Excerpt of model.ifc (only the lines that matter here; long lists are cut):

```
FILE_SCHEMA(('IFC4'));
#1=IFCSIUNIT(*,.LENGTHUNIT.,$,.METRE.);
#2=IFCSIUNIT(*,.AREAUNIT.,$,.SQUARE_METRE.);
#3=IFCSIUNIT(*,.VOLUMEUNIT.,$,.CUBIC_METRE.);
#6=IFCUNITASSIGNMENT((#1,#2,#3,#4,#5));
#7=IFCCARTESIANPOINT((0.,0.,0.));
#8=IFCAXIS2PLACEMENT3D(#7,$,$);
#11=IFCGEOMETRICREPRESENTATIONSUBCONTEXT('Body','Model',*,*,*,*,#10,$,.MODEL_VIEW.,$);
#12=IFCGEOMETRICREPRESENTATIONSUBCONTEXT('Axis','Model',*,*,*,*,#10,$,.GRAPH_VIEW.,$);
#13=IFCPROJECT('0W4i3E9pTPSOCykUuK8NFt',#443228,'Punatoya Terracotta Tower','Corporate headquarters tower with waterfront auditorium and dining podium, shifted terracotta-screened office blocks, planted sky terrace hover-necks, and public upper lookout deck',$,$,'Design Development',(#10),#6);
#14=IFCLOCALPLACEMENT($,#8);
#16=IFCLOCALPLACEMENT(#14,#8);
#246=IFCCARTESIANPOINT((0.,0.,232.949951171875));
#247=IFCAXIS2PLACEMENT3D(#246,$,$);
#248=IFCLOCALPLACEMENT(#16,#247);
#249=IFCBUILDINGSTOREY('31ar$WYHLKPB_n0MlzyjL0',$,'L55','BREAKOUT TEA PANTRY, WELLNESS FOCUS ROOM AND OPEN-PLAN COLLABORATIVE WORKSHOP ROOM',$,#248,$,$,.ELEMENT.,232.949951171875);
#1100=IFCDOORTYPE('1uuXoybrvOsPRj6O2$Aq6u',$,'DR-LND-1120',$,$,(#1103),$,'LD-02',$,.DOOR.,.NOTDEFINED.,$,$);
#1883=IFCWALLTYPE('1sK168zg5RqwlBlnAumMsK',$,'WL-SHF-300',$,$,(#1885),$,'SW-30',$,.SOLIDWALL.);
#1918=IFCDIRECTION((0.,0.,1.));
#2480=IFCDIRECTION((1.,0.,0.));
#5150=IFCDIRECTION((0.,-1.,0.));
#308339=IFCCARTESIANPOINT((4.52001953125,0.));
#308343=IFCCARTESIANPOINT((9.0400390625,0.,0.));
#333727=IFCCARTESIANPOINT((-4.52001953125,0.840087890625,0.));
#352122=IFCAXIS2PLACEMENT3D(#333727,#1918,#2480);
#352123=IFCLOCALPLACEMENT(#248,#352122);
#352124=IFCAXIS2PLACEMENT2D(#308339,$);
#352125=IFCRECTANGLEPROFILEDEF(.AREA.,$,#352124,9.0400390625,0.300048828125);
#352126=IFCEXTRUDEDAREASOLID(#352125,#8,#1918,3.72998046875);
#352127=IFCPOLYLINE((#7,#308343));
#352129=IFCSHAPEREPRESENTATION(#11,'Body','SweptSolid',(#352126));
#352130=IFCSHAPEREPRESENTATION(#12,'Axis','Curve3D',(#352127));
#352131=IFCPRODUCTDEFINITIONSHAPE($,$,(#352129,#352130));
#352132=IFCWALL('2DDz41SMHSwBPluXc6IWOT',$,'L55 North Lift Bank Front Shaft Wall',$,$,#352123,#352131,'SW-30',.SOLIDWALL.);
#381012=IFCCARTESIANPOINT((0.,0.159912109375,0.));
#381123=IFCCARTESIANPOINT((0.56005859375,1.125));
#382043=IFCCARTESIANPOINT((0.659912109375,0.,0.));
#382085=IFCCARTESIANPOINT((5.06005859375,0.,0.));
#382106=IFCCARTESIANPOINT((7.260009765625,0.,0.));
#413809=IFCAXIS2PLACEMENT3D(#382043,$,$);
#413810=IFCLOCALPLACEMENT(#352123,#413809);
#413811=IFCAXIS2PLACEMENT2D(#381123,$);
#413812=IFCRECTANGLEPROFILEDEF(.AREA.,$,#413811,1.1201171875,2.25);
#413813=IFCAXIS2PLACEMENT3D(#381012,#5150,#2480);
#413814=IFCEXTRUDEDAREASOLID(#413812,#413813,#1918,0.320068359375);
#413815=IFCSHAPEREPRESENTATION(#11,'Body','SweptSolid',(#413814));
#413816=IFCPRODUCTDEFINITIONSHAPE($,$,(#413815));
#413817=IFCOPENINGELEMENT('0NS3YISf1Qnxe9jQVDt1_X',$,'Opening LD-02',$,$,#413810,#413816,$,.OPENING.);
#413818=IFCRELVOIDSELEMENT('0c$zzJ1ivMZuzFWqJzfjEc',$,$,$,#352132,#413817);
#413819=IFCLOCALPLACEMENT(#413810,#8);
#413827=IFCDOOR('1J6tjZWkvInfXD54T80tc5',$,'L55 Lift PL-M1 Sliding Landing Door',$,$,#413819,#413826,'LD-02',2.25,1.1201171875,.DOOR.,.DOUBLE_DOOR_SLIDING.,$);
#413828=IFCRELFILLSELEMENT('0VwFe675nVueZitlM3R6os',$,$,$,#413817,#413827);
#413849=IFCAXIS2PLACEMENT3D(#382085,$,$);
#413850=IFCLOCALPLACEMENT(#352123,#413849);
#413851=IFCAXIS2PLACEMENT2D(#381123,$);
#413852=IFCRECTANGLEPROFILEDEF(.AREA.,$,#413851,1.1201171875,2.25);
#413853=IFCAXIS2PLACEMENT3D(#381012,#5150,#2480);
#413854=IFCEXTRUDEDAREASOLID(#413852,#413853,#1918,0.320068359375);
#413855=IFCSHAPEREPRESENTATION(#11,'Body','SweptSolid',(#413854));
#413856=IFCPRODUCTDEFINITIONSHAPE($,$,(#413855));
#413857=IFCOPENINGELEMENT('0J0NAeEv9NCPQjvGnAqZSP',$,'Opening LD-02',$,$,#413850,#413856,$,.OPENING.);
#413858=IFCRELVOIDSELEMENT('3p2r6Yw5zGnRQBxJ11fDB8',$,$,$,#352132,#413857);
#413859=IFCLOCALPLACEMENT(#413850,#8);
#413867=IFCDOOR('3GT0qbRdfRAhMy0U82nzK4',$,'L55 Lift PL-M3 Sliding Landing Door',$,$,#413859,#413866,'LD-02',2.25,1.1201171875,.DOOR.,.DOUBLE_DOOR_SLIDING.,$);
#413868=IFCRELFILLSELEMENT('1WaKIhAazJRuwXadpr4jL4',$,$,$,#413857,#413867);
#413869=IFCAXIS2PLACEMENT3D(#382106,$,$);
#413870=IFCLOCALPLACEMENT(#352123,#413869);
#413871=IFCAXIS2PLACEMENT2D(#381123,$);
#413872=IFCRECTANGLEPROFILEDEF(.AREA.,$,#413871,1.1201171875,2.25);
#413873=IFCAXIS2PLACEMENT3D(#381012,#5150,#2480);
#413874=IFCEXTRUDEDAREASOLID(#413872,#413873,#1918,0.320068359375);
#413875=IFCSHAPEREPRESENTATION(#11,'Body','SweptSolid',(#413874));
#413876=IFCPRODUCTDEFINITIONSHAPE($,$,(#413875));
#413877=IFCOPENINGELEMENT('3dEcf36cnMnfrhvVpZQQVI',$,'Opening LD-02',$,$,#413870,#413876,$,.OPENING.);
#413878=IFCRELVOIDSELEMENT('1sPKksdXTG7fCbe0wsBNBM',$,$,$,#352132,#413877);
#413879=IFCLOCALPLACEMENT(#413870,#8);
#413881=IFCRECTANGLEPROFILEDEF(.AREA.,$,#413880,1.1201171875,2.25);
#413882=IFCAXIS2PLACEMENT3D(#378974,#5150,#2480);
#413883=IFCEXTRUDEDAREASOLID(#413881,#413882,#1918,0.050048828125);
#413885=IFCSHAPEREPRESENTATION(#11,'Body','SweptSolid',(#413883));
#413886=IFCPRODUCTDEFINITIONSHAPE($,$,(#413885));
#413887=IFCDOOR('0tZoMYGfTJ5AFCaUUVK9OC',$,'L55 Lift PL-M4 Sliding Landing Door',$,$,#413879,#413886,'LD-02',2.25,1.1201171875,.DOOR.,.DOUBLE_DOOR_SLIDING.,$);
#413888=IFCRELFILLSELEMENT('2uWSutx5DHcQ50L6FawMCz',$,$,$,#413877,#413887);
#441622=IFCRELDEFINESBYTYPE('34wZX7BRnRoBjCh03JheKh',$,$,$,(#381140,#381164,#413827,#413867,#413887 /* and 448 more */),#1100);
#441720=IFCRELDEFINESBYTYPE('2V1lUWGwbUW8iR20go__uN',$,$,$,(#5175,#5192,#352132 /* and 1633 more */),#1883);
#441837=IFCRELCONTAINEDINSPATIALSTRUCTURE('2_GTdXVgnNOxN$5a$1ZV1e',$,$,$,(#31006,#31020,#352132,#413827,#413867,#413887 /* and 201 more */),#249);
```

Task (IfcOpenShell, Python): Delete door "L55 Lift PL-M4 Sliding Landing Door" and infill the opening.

```python
import ifcopenshell
import ifcopenshell.api.feature
import ifcopenshell.api.root
import ifcopenshell.geom
import ifcopenshell.util.shape

model = ifcopenshell.open("model.ifc")
settings = ifcopenshell.geom.settings()


def volume(element):
    """Net volume in cubic metres, openings subtracted."""
    shape = ifcopenshell.geom.create_shape(settings, element)
    return ifcopenshell.util.shape.get_volume(shape.geometry)


door = model.by_guid("0tZoMYGfTJ5AFCaUUVK9OC")
opening = door.FillsVoids[0].RelatingOpeningElement
wall = opening.VoidsElements[0].RelatingBuildingElement
before = volume(wall)

ifcopenshell.api.root.remove_product(model, product=door)
ifcopenshell.api.feature.remove_feature(model, feature=opening)

after = volume(wall)

print(f"wall volume {before:.3f} -> {after:.3f} m3")

model.write("model_rev.ifc")
```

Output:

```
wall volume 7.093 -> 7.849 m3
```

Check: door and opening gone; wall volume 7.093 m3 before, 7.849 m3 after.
